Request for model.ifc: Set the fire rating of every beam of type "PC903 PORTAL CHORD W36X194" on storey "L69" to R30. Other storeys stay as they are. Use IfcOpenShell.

First a look at what the model holds.

```python
import ifcopenshell
import ifcopenshell.util.element

model = ifcopenshell.open("model.ifc")
print(model.schema)
storey = next(s for s in model.by_type("IfcBuildingStorey") if s.Name == "L69")
beams = [e for e in ifcopenshell.util.element.get_decomposition(storey) if e.is_a("IfcBeam")]
seen = {}
for e in beams:
    element_type = ifcopenshell.util.element.get_type(e)
    key = (element_type.Name if element_type != e and element_type else None, ifcopenshell.util.element.get_pset(e, "Pset_BeamCommon", "FireRating"))
    seen[key] = seen.get(key, 0) + 1
for (name, value), count in sorted(seen.items(), key=str):
    print(count, "x", name, "|", value)
```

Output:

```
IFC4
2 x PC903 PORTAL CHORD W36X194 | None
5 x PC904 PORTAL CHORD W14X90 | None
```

```python
import ifcopenshell
import ifcopenshell.api.pset
import ifcopenshell.util.element

model = ifcopenshell.open("model.ifc")

storey = next(s for s in model.by_type("IfcBuildingStorey") if s.Name == "L69")
beams = [e for e in ifcopenshell.util.element.get_decomposition(storey) if e.is_a("IfcBeam")]

count = 0
for e in beams:
    element_type = ifcopenshell.util.element.get_type(e)
    if element_type in (None, e) or element_type.Name != "PC903 PORTAL CHORD W36X194":
        continue
    found = ifcopenshell.util.element.get_pset(e, "Pset_BeamCommon", should_inherit=False)
    if found:
        pset = model.by_id(found["id"])
        if len(ifcopenshell.util.element.get_elements_by_pset(pset)) > 1:
            pset = ifcopenshell.api.pset.unshare_pset(model, products=[e], pset=pset)[0]
    else:
        pset = ifcopenshell.api.pset.add_pset(model, product=e, name="Pset_BeamCommon")
    ifcopenshell.api.pset.edit_pset(model, pset=pset, properties={"FireRating": "R30"})
    count += 1

print(count, "beams updated")

model.write("model_v2.ifc")
```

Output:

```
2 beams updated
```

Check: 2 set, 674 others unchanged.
